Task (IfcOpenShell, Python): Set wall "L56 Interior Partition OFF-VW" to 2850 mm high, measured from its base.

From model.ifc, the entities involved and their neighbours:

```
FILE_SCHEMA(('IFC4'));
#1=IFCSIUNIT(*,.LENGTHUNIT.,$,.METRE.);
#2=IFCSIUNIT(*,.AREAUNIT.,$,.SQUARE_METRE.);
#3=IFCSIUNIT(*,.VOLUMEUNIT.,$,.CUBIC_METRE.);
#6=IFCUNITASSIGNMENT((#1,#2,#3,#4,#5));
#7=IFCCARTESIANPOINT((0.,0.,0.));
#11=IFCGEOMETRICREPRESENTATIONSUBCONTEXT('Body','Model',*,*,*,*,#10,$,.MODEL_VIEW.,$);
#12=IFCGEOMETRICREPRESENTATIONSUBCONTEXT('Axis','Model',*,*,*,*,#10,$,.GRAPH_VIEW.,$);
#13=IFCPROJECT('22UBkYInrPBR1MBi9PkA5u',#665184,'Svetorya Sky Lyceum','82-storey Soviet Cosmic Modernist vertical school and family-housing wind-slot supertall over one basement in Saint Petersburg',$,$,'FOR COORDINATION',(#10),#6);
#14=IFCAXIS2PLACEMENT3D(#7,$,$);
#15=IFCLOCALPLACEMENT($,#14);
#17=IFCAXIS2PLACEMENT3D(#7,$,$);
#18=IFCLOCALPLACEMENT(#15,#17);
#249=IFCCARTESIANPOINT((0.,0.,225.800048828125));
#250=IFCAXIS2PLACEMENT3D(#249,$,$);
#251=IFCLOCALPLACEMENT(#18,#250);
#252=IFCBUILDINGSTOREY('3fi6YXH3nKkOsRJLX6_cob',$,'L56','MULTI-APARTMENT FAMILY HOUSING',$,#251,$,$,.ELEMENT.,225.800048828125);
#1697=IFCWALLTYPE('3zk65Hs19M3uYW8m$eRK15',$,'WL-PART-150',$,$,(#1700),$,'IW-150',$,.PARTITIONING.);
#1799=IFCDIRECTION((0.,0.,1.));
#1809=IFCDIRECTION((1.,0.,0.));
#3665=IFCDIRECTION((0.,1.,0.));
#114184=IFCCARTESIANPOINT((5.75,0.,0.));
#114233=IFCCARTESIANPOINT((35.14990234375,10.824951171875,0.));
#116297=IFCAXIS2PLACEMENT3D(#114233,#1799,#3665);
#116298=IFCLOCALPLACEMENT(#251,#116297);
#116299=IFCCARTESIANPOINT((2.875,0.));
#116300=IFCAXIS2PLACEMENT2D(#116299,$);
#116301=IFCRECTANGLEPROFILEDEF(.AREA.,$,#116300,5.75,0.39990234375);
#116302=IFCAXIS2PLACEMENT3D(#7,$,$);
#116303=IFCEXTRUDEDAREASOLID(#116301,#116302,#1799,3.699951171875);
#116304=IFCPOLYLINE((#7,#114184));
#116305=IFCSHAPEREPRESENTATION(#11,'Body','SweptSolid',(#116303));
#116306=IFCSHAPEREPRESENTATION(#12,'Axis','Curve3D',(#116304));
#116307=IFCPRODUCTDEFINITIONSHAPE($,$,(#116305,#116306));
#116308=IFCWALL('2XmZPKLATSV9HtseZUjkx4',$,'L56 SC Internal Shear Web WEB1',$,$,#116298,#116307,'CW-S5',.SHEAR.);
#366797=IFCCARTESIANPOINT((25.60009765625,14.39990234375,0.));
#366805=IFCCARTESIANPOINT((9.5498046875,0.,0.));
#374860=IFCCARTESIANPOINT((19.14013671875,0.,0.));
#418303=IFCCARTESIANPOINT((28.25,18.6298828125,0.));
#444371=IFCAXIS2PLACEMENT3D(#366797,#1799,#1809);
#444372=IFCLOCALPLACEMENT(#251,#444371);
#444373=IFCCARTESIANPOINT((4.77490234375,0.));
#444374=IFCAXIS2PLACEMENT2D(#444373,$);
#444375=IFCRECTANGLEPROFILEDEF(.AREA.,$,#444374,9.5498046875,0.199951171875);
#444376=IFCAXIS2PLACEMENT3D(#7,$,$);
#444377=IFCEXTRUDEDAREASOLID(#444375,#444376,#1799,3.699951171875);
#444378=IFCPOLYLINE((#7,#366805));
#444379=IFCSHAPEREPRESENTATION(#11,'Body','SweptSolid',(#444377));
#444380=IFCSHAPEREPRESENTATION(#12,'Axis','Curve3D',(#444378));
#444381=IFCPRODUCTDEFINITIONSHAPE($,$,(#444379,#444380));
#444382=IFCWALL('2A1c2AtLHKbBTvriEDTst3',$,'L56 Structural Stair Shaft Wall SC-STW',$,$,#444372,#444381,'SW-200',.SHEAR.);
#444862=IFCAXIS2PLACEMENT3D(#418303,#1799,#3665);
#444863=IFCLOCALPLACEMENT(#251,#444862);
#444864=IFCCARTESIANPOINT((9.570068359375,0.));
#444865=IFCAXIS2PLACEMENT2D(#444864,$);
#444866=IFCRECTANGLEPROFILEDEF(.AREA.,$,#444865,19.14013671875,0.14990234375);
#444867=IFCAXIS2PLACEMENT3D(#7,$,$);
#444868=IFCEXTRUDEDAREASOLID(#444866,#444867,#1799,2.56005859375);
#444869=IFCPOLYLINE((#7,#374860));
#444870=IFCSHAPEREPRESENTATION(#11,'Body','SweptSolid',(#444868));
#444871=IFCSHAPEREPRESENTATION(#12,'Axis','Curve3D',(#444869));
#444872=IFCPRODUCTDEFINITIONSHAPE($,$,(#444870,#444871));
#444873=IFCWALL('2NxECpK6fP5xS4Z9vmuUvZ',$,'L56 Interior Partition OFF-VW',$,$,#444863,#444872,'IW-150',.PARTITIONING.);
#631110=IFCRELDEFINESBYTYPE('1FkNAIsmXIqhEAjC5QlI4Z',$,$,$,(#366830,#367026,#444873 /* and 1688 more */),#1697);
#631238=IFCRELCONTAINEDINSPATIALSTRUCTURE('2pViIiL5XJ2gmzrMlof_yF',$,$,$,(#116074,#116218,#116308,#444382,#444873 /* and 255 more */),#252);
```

```python
import ifcopenshell
import ifcopenshell.geom
import ifcopenshell.util.representation
import ifcopenshell.util.shape
import ifcopenshell.util.unit

model = ifcopenshell.open("model.ifc")
unit_scale = ifcopenshell.util.unit.calculate_unit_scale(model)
settings = ifcopenshell.geom.settings()


def volume(element):
    """Net volume in cubic metres, openings subtracted."""
    shape = ifcopenshell.geom.create_shape(settings, element)
    return ifcopenshell.util.shape.get_volume(shape.geometry)


wall = model.by_id(444873)
before = volume(wall)

body = ifcopenshell.util.representation.get_representation(wall, "Model", "Body")
solid = body.Items[0]
old_height = solid.Depth
solid.Depth = 2.85 / unit_scale
after = volume(wall)

print(f"height {old_height:g} -> {solid.Depth:g}, volume {before:.3f} -> {after:.3f} m3")

model.write("model_rev.ifc")
```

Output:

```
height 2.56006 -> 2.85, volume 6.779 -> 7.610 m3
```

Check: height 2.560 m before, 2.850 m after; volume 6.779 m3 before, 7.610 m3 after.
